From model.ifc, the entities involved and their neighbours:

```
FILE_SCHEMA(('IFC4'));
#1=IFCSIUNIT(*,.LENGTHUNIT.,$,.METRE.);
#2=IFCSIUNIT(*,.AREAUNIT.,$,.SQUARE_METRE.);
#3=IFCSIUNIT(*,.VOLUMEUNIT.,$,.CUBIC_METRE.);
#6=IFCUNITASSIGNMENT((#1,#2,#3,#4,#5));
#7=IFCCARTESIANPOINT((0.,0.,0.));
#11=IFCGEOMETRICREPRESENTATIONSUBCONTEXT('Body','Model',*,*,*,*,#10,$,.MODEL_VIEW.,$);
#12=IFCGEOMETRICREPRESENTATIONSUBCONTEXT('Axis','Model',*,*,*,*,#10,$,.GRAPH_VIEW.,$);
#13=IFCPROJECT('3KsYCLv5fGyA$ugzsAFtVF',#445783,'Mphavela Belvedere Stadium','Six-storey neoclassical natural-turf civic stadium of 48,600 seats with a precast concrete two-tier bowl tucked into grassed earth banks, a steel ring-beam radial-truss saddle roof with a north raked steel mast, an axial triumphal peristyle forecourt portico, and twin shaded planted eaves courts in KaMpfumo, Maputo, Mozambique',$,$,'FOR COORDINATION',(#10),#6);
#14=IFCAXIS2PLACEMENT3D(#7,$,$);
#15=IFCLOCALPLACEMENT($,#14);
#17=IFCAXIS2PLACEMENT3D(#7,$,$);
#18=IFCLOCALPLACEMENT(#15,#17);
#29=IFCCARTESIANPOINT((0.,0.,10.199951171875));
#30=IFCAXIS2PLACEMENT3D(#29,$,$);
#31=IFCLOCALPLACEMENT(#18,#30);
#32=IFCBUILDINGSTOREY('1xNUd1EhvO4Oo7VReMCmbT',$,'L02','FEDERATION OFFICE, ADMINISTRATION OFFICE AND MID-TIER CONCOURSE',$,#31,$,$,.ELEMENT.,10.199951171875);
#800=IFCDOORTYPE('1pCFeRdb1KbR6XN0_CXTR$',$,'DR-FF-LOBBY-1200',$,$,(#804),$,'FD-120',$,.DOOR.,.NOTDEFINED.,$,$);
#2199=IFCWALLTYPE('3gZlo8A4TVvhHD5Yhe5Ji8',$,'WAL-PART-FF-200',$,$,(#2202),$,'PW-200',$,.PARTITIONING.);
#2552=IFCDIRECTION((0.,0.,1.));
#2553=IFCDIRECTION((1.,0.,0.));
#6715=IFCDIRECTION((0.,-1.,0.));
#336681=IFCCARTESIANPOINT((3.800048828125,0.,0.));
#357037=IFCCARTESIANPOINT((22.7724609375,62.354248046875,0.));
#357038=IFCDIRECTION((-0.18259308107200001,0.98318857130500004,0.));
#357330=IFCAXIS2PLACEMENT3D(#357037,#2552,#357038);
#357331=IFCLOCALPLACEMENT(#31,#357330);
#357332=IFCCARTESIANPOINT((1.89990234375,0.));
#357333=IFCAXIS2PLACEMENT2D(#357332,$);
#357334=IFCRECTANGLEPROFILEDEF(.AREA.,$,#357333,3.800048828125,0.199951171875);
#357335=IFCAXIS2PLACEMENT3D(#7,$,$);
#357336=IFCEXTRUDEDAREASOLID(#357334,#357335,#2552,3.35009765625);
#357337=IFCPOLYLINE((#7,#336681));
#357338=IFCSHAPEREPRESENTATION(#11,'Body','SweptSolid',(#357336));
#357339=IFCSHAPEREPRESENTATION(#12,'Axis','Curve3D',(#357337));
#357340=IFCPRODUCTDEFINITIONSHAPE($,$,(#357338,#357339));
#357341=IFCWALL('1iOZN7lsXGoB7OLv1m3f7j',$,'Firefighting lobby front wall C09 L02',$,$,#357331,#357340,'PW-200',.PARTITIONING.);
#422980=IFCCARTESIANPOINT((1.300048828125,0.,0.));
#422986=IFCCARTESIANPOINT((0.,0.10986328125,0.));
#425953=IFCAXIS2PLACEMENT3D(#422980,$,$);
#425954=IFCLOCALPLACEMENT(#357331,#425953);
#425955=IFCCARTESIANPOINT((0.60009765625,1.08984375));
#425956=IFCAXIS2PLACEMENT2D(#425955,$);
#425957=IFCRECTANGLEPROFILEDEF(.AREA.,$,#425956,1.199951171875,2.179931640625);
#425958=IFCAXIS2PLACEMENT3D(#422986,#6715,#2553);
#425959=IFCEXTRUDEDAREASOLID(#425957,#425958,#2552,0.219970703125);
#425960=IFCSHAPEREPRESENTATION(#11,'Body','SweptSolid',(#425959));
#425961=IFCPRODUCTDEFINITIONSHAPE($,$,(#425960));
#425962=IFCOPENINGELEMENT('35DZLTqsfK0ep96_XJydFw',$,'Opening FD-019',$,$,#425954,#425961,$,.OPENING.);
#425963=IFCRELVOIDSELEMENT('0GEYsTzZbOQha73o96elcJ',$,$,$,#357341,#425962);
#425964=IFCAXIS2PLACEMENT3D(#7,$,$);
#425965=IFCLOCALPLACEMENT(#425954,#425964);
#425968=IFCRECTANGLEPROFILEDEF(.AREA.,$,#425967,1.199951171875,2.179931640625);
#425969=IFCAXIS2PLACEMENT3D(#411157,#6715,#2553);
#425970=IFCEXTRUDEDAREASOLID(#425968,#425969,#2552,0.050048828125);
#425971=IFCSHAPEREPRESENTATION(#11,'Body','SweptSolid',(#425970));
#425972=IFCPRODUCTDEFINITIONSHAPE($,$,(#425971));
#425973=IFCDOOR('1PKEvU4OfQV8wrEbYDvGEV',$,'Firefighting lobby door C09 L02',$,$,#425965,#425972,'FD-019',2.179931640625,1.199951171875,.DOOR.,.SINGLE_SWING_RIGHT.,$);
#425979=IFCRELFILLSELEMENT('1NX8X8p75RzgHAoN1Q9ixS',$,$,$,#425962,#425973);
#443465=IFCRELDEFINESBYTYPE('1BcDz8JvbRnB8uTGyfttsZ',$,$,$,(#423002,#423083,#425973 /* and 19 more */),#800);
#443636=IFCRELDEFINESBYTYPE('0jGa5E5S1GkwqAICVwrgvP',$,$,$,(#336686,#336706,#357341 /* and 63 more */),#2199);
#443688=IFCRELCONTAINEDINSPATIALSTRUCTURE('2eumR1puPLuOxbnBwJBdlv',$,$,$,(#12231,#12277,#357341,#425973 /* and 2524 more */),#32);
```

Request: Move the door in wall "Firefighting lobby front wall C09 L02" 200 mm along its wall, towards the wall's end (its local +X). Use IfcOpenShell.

```python
import ifcopenshell
import ifcopenshell.api.geometry
import ifcopenshell.util.placement
import ifcopenshell.util.unit

model = ifcopenshell.open("model.ifc")
unit_scale = ifcopenshell.util.unit.calculate_unit_scale(model)

door = model.by_guid("1PKEvU4OfQV8wrEbYDvGEV")
opening = door.FillsVoids[0].RelatingOpeningElement
wall = opening.VoidsElements[0].RelatingBuildingElement

wall_matrix = ifcopenshell.util.placement.get_local_placement(wall.ObjectPlacement)
shift = wall_matrix[:3, 0] * 0.2 / unit_scale
before = ifcopenshell.util.placement.get_local_placement(door.ObjectPlacement)[:3, 3].copy()

# The door is placed relative to its opening, so it follows when the opening moves.
matrix = ifcopenshell.util.placement.get_local_placement(opening.ObjectPlacement)
matrix[:3, 3] += shift
ifcopenshell.api.geometry.edit_object_placement(
    model, product=opening, matrix=matrix, is_si=False, should_transform_children=True
)

after = ifcopenshell.util.placement.get_local_placement(door.ObjectPlacement)[:3, 3]
print("door moved by", (after - before).round(3) + 0.0)

model.write("model_v2.ifc")
```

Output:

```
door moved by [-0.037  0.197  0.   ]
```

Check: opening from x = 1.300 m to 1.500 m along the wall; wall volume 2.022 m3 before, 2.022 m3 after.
